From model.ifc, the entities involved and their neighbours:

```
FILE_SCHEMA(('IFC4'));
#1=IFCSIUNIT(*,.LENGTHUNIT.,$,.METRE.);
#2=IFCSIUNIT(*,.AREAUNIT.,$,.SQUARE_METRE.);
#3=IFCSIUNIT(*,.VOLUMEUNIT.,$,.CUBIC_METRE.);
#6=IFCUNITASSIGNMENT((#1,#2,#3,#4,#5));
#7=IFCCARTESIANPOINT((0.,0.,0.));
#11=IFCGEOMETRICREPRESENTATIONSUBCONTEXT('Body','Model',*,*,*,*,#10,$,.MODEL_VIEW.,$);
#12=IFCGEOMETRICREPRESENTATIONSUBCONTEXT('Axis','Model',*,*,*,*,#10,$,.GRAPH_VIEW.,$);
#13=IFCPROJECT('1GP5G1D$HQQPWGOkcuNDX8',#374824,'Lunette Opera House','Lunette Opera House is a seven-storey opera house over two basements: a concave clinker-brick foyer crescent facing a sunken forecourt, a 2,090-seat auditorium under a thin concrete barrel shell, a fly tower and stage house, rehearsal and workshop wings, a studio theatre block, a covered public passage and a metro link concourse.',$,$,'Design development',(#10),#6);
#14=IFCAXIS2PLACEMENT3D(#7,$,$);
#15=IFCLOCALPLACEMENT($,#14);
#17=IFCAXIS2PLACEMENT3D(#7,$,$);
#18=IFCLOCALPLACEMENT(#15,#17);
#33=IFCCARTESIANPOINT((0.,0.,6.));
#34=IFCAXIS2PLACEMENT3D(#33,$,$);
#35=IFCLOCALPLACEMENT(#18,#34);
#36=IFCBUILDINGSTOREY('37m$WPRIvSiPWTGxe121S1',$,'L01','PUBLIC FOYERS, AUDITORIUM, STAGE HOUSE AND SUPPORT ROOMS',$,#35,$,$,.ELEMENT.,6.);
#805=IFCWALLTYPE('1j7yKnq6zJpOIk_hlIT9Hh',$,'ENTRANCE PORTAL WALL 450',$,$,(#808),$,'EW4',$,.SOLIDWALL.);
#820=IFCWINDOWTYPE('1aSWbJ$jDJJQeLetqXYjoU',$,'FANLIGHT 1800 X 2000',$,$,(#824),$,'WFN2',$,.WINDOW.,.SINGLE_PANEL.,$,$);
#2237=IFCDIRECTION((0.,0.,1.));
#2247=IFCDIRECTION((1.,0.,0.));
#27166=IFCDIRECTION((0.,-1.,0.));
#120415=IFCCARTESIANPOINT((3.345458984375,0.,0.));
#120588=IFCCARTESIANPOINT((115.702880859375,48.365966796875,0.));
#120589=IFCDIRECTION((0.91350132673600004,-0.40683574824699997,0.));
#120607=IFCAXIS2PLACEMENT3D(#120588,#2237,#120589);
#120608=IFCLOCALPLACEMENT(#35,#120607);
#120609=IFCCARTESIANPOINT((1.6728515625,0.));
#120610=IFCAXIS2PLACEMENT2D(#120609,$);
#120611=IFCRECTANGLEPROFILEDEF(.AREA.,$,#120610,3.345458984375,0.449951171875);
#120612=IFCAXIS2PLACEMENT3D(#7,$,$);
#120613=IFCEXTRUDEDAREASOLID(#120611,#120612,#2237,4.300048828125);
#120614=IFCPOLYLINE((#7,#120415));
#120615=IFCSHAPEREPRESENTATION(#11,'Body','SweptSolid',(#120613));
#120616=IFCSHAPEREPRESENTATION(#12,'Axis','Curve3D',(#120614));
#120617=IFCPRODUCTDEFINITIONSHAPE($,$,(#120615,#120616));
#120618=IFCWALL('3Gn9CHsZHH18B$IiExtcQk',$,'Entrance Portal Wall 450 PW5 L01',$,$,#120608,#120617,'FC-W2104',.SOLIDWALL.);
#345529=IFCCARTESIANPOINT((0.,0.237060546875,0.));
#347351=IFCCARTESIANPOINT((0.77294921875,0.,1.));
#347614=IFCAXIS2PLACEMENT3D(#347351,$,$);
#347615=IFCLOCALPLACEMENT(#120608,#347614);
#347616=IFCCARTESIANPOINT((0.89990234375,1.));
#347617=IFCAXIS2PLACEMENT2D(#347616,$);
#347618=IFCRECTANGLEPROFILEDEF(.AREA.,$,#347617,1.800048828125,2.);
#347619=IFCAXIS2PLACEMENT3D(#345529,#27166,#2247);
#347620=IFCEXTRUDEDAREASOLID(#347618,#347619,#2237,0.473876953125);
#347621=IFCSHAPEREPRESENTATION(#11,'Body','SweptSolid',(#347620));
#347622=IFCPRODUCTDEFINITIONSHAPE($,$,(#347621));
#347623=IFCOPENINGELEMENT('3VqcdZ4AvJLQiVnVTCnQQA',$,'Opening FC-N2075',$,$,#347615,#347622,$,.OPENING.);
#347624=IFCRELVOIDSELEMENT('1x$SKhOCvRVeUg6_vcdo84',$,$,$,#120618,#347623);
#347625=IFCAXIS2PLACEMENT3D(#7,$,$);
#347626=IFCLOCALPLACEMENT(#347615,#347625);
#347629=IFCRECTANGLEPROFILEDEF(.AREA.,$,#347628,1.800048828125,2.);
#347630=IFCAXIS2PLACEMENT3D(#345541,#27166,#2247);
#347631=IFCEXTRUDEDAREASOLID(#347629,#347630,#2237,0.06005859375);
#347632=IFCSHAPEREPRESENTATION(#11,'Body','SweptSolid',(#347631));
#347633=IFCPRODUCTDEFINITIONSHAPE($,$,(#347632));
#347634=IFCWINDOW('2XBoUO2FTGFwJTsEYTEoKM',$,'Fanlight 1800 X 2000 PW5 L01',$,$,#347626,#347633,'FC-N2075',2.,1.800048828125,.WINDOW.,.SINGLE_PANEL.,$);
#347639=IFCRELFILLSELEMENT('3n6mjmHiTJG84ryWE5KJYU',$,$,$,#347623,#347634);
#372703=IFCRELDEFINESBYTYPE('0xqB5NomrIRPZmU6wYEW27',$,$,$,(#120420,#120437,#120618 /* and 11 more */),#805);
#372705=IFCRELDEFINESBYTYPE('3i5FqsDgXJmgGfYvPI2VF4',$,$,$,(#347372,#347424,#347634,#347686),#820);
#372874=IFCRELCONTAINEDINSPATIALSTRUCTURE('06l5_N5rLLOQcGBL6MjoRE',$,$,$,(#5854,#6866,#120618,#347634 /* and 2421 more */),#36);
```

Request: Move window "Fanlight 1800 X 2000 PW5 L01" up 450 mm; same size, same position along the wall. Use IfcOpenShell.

```python
import numpy as np
import ifcopenshell
import ifcopenshell.api.geometry
import ifcopenshell.util.placement
import ifcopenshell.util.unit

model = ifcopenshell.open("model.ifc")
unit_scale = ifcopenshell.util.unit.calculate_unit_scale(model)

window = model.by_id(347634)
opening = window.FillsVoids[0].RelatingOpeningElement
dz = 0.45 / unit_scale

shift = np.array([0.0, 0.0, dz])
# The window is placed relative to its opening, so it follows when the opening moves.
matrix = ifcopenshell.util.placement.get_local_placement(opening.ObjectPlacement)
matrix[:3, 3] += shift
ifcopenshell.api.geometry.edit_object_placement(
    model, product=opening, matrix=matrix, is_si=False, should_transform_children=True
)

print(f"moved by {dz * unit_scale:+.3f} m")

model.write("model_edited.ifc")
```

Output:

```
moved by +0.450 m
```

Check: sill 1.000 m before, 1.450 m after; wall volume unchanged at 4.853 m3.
